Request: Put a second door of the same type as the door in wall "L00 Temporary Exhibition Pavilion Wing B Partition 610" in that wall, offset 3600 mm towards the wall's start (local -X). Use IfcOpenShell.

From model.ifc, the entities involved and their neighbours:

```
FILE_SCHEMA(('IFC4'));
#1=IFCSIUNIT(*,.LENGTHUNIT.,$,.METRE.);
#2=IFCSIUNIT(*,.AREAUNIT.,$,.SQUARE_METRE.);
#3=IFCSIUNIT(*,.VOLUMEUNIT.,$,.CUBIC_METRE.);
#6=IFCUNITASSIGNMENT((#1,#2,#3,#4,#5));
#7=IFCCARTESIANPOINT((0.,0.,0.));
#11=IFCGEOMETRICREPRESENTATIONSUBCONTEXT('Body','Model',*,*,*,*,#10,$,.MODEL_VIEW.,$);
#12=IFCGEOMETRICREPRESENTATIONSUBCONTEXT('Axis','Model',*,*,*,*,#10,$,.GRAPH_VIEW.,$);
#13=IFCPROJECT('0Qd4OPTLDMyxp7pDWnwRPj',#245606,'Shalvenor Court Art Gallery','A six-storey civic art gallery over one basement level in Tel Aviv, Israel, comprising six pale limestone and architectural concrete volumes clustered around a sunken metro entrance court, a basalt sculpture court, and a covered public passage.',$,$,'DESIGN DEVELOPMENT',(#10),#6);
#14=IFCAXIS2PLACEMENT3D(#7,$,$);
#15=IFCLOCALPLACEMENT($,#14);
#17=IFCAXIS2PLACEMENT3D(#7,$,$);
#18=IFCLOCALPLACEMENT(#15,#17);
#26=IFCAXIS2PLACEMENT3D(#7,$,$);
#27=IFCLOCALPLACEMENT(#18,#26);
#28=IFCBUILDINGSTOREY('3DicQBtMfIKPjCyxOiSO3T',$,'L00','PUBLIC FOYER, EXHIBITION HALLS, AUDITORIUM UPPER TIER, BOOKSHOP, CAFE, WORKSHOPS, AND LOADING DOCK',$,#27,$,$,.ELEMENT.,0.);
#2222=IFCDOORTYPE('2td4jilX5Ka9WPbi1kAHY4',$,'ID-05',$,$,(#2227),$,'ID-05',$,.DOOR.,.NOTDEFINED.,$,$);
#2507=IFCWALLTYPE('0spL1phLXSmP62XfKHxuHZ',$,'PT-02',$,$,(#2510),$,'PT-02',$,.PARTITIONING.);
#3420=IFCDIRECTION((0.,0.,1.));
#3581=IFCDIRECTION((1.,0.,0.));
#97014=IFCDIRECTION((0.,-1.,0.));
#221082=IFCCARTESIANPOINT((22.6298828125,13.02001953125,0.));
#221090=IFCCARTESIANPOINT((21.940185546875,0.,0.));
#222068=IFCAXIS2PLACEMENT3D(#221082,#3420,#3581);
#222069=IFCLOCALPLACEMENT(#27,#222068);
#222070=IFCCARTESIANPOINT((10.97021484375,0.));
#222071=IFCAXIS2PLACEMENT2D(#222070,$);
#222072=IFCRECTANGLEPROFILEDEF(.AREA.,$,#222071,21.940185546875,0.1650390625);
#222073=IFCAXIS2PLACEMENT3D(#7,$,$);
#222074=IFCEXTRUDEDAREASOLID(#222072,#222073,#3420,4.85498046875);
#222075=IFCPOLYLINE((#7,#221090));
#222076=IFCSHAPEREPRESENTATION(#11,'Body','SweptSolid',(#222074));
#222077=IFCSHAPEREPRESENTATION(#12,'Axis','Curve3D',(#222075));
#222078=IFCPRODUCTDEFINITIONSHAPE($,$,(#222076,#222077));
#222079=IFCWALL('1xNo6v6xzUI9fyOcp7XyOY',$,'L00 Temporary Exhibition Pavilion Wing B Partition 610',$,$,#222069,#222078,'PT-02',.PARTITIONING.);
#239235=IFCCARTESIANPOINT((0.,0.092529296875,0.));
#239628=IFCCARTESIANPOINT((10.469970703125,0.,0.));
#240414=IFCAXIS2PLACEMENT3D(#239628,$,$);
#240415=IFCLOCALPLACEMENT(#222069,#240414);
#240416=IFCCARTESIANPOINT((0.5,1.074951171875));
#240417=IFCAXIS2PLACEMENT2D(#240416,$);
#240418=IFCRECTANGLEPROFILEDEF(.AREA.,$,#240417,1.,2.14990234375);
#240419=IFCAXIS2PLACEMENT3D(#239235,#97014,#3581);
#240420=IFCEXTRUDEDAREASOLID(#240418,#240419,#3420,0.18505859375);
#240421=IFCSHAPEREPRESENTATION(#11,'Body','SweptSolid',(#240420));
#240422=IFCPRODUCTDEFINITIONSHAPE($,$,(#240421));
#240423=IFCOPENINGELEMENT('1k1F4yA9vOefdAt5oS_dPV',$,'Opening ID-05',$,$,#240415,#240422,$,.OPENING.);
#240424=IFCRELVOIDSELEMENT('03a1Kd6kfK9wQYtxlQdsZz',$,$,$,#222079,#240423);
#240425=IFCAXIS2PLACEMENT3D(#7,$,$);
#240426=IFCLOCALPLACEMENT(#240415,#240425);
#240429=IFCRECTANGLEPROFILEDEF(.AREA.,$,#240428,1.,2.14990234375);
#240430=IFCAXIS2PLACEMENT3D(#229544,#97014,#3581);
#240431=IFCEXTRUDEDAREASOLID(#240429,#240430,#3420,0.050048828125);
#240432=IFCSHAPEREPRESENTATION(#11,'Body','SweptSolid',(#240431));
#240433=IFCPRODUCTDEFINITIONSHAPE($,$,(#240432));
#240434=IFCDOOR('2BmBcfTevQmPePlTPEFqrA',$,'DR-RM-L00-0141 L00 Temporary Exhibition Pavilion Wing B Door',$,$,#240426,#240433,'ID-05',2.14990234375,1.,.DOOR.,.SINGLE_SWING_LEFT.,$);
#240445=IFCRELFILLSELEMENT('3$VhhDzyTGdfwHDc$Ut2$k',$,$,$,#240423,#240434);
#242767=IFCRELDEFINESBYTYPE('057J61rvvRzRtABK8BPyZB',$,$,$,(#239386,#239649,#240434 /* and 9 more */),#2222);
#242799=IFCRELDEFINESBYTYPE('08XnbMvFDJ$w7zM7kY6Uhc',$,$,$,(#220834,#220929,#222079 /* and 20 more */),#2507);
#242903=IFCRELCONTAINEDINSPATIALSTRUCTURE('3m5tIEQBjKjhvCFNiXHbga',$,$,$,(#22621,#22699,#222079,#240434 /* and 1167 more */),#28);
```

```python
import ifcopenshell
import ifcopenshell.api.feature
import ifcopenshell.api.geometry
import ifcopenshell.api.root
import ifcopenshell.geom
import ifcopenshell.util.element
import ifcopenshell.util.placement
import ifcopenshell.util.shape

model = ifcopenshell.open("model.ifc")
settings = ifcopenshell.geom.settings()


def volume(element):
    """Net volume in cubic metres, openings subtracted."""
    shape = ifcopenshell.geom.create_shape(settings, element)
    return ifcopenshell.util.shape.get_volume(shape.geometry)


door = model.by_guid("2BmBcfTevQmPePlTPEFqrA")
opening = door.FillsVoids[0].RelatingOpeningElement
wall = opening.VoidsElements[0].RelatingBuildingElement
before = volume(wall)
shift = ifcopenshell.util.placement.get_local_placement(wall.ObjectPlacement)[:3, 0] * -3.6

# copy_class copies the void relationship, type, container and properties, but no geometry.
new_opening = ifcopenshell.api.root.copy_class(model, product=opening)
new_opening.Representation = ifcopenshell.util.element.copy_deep(
    model, opening.Representation, exclude=["IfcGeometricRepresentationContext", "IfcRepresentationMap"]
)
new_door = ifcopenshell.api.root.copy_class(model, product=door)
new_door.Representation = ifcopenshell.util.element.copy_deep(
    model, door.Representation, exclude=["IfcGeometricRepresentationContext", "IfcRepresentationMap"]
)
new_door.Tag = None
ifcopenshell.api.feature.add_filling(model, opening=new_opening, element=new_door)

for old, new in ((opening, new_opening), (door, new_door)):
    matrix = ifcopenshell.util.placement.get_local_placement(old.ObjectPlacement)
    matrix[:3, 3] += shift
    ifcopenshell.api.geometry.edit_object_placement(model, product=new, matrix=matrix, is_si=False)

after = volume(wall)

print(f"wall volume {before:.3f} -> {after:.3f} m3")

model.write("model_rev.ifc")
```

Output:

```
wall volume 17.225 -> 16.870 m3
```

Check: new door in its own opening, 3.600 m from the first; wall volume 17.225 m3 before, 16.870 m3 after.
